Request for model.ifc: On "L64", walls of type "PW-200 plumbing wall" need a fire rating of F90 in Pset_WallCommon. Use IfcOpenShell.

First a look at what the model holds.

```python
import ifcopenshell
import ifcopenshell.util.element

model = ifcopenshell.open("model.ifc")
print(model.schema)
storey = next(s for s in model.by_type("IfcBuildingStorey") if s.Name == "L64")
walls = [e for e in ifcopenshell.util.element.get_decomposition(storey) if e.is_a("IfcWall")]
seen = {}
for e in walls:
    element_type = ifcopenshell.util.element.get_type(e)
    key = (element_type.Name if element_type != e and element_type else None, ifcopenshell.util.element.get_pset(e, "Pset_WallCommon", "FireRating"))
    seen[key] = seen.get(key, 0) + 1
for (name, value), count in sorted(seen.items(), key=str):
    print(count, "x", name, "|", value)
```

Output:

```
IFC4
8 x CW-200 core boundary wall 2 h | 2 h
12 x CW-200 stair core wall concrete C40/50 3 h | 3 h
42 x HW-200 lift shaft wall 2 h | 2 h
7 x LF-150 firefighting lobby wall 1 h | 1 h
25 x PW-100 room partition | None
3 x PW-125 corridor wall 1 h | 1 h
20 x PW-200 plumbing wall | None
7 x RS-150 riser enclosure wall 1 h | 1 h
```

```python
import ifcopenshell
import ifcopenshell.api.pset
import ifcopenshell.util.element

model = ifcopenshell.open("model.ifc")

storey = next(s for s in model.by_type("IfcBuildingStorey") if s.Name == "L64")
walls = [e for e in ifcopenshell.util.element.get_decomposition(storey) if e.is_a("IfcWall")]

count = 0
for e in walls:
    element_type = ifcopenshell.util.element.get_type(e)
    if element_type in (None, e) or element_type.Name != "PW-200 plumbing wall":
        continue
    found = ifcopenshell.util.element.get_pset(e, "Pset_WallCommon", should_inherit=False)
    if found:
        pset = model.by_id(found["id"])
        if len(ifcopenshell.util.element.get_elements_by_pset(pset)) > 1:
            pset = ifcopenshell.api.pset.unshare_pset(model, products=[e], pset=pset)[0]
    else:
        pset = ifcopenshell.api.pset.add_pset(model, product=e, name="Pset_WallCommon")
    ifcopenshell.api.pset.edit_pset(model, pset=pset, properties={"FireRating": "F90"})
    count += 1

print(count, "walls updated")

model.write("model_edited.ifc")
```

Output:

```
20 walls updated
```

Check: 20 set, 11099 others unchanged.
